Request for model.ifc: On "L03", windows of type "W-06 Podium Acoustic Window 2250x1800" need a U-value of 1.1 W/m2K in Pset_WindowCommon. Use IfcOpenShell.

First a look at what the model holds.

```python
import ifcopenshell
import ifcopenshell.util.element

model = ifcopenshell.open("model.ifc")
print(model.schema)
storey = next(s for s in model.by_type("IfcBuildingStorey") if s.Name == "L03")
windows = [e for e in ifcopenshell.util.element.get_decomposition(storey) if e.is_a("IfcWindow")]
seen = {}
for e in windows:
    element_type = ifcopenshell.util.element.get_type(e)
    key = (element_type.Name if element_type != e and element_type else None, ifcopenshell.util.element.get_pset(e, "Pset_WindowCommon", "ThermalTransmittance"))
    seen[key] = seen.get(key, 0) + 1
for (name, value), count in sorted(seen.items(), key=str):
    print(count, "x", name, "|", value)
```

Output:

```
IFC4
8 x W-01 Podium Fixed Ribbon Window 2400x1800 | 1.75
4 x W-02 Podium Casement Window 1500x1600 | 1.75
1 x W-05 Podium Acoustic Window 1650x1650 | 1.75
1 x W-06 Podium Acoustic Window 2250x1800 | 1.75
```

```python
import ifcopenshell
import ifcopenshell.api.pset
import ifcopenshell.util.element

model = ifcopenshell.open("model.ifc")

storey = next(s for s in model.by_type("IfcBuildingStorey") if s.Name == "L03")
windows = [e for e in ifcopenshell.util.element.get_decomposition(storey) if e.is_a("IfcWindow")]

count = 0
for e in windows:
    element_type = ifcopenshell.util.element.get_type(e)
    if element_type in (None, e) or element_type.Name != "W-06 Podium Acoustic Window 2250x1800":
        continue
    # add_pset returns the element's existing set when there is one.
    pset = ifcopenshell.api.pset.add_pset(model, product=e, name="Pset_WindowCommon")
    ifcopenshell.api.pset.edit_pset(model, pset=pset, properties={"ThermalTransmittance": 1.1})
    count += 1

print(count, "windows updated")

model.write("model_v2.ifc")
```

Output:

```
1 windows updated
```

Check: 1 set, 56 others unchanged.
